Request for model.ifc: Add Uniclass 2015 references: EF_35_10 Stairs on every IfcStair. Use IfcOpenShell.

First a look at what the model holds.

```python
import ifcopenshell

model = ifcopenshell.open("model.ifc")
print(model.schema)
print("classifications:", [c.Name for c in model.by_type("IfcClassification")])
for ifc_class in ("IfcDoor", "IfcRoof", "IfcStair", "IfcWall", "IfcWindow"):
    print(ifc_class, len(model.by_type(ifc_class)))
```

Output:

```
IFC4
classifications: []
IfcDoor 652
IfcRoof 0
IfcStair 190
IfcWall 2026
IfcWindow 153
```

```python
import ifcopenshell
import ifcopenshell.api.classification

model = ifcopenshell.open("model.ifc")

system = ifcopenshell.api.classification.add_classification(model, classification="Uniclass 2015")

codes = {
    "IfcStair": ("EF_35_10", "Stairs"),
}
for ifc_class, (code, name) in codes.items():
    products = model.by_type(ifc_class)
    ifcopenshell.api.classification.add_reference(
        model, products=products, classification=system, identification=code, name=name
    )
    print(code, len(products))

model.write("model-out.ifc")
```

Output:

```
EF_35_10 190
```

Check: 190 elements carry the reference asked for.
